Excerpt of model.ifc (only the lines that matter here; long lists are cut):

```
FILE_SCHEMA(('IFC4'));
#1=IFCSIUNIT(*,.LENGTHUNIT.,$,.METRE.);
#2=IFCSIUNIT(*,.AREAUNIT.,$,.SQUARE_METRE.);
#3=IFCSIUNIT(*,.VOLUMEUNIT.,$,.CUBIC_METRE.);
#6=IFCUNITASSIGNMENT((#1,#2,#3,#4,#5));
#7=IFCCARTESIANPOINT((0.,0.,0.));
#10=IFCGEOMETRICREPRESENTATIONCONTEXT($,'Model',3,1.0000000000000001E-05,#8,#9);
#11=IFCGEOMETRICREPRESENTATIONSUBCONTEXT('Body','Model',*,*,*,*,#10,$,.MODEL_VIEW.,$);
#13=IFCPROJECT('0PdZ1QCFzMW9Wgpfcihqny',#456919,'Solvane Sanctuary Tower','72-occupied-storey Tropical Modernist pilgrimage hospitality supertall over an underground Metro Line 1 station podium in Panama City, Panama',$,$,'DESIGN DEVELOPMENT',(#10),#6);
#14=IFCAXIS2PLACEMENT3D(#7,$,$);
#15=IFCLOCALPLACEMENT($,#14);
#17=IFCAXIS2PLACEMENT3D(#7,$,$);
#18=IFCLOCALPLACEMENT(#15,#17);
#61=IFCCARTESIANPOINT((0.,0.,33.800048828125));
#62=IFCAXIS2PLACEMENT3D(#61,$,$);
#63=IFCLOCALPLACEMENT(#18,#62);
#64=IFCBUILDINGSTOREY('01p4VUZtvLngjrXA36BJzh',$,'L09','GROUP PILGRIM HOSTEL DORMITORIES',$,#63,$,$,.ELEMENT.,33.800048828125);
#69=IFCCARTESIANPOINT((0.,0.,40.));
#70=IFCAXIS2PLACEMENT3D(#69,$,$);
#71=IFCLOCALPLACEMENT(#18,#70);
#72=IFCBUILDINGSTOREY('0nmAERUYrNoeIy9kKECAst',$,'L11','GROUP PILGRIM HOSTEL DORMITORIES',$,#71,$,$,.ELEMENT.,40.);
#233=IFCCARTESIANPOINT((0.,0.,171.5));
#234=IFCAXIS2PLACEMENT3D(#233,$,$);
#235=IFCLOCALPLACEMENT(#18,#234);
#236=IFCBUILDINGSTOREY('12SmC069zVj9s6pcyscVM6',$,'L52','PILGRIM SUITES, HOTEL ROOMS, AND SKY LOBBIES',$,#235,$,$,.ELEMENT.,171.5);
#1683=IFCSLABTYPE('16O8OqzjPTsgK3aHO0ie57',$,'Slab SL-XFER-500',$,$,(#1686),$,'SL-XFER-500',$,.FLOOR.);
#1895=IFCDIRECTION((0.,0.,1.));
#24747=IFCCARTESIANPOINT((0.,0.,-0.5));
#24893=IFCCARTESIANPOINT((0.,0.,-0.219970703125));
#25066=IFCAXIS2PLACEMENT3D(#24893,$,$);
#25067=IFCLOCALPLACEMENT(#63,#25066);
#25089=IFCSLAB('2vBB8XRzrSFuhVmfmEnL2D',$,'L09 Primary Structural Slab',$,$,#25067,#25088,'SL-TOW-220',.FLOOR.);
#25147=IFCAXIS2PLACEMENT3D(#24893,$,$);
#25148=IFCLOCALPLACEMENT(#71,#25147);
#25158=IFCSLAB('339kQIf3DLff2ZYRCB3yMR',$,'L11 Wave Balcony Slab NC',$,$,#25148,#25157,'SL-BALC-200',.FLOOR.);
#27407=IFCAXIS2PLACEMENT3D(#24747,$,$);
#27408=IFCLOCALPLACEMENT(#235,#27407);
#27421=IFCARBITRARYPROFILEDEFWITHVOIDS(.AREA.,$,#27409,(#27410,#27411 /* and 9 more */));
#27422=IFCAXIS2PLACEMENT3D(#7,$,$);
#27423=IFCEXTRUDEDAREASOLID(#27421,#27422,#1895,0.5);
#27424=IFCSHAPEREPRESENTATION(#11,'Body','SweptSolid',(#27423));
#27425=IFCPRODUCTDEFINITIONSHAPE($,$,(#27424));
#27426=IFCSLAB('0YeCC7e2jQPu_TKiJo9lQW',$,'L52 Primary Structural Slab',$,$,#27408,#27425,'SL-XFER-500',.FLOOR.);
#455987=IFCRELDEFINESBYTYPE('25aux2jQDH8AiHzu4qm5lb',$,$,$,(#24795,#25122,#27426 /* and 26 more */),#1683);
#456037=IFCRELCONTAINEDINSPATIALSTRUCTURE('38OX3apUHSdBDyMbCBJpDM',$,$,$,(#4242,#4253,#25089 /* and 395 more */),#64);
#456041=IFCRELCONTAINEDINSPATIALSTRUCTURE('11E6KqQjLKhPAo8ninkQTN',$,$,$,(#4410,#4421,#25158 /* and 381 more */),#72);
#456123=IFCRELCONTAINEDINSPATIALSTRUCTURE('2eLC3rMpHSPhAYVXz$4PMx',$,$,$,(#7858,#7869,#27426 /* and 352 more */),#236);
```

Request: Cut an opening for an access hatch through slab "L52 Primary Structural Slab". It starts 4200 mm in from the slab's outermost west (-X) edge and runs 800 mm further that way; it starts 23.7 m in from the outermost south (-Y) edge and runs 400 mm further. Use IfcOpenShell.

```python
import numpy as np
import ifcopenshell
import ifcopenshell.api.feature
import ifcopenshell.api.geometry
import ifcopenshell.api.root
import ifcopenshell.geom
import ifcopenshell.util.placement
import ifcopenshell.util.representation
import ifcopenshell.util.shape
import ifcopenshell.util.unit

model = ifcopenshell.open("model.ifc")
unit_scale = ifcopenshell.util.unit.calculate_unit_scale(model)
settings = ifcopenshell.geom.settings()


def volume(element):
    """Net volume in cubic metres, openings subtracted."""
    shape = ifcopenshell.geom.create_shape(settings, element)
    return ifcopenshell.util.shape.get_volume(shape.geometry)


slab = model.by_id(27426)
before = volume(slab)

# Extent in the slab's own axes, in metres. The edges named are its -X and -Y sides.
slab_shape = ifcopenshell.geom.create_shape(settings, slab)
vertices = ifcopenshell.util.shape.get_vertices(slab_shape.geometry)
x_min, y_min, bottom = vertices.min(axis=0)
top = vertices[:, 2].max()

opening = ifcopenshell.api.root.create_entity(model, ifc_class="IfcOpeningElement", name="Access hatch opening", predefined_type="OPENING")
context = ifcopenshell.util.representation.get_context(model, "Model", "Body", "MODEL_VIEW")
width, depth = 0.8, 0.4
outline = [(0.0, 0.0), (width, 0.0), (width, depth), (0.0, depth), (0.0, 0.0)]
# Overshoot both faces by 50 mm so the cut is clean.
shape = ifcopenshell.api.geometry.add_slab_representation(
    model, context=context, depth=top - bottom + 0.1, polyline=outline
)
ifcopenshell.api.geometry.assign_representation(model, product=opening, representation=shape)

matrix = ifcopenshell.util.placement.get_local_placement(slab.ObjectPlacement)
matrix[:, 3] = matrix @ np.append(np.array([x_min + 4.2, y_min + 23.7, bottom - 0.05]) / unit_scale, 1.0)
ifcopenshell.api.geometry.edit_object_placement(model, product=opening, matrix=matrix, is_si=False)
ifcopenshell.api.feature.add_feature(model, feature=opening, element=slab)

after = volume(slab)

print(f"slab volume {before:.3f} -> {after:.3f} m3")

model.write("model_rev.ifc")
```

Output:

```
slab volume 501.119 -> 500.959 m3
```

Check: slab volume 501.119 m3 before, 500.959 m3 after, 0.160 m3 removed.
